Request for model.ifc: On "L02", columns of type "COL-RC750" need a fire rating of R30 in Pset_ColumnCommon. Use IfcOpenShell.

First a look at what the model holds.

```python
import ifcopenshell
import ifcopenshell.util.element

model = ifcopenshell.open("model.ifc")
print(model.schema)
storey = next(s for s in model.by_type("IfcBuildingStorey") if s.Name == "L02")
columns = [e for e in ifcopenshell.util.element.get_decomposition(storey) if e.is_a("IfcColumn")]
seen = {}
for e in columns:
    element_type = ifcopenshell.util.element.get_type(e)
    key = (element_type.Name if element_type != e and element_type else None, ifcopenshell.util.element.get_pset(e, "Pset_ColumnCommon", "FireRating"))
    seen[key] = seen.get(key, 0) + 1
for (name, value), count in sorted(seen.items(), key=str):
    print(count, "x", name, "|", value)
```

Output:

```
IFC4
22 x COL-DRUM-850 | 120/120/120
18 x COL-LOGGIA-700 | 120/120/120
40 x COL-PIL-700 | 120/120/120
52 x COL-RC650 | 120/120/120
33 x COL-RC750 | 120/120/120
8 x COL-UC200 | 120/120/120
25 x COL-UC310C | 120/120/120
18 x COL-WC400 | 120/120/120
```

```python
import ifcopenshell
import ifcopenshell.api.pset
import ifcopenshell.util.element

model = ifcopenshell.open("model.ifc")

storey = next(s for s in model.by_type("IfcBuildingStorey") if s.Name == "L02")
columns = [e for e in ifcopenshell.util.element.get_decomposition(storey) if e.is_a("IfcColumn")]

count = 0
for e in columns:
    element_type = ifcopenshell.util.element.get_type(e)
    if element_type in (None, e) or element_type.Name != "COL-RC750":
        continue
    # add_pset returns the element's existing set when there is one.
    pset = ifcopenshell.api.pset.add_pset(model, product=e, name="Pset_ColumnCommon")
    ifcopenshell.api.pset.edit_pset(model, pset=pset, properties={"FireRating": "R30"})
    count += 1

print(count, "columns updated")

model.write("model_rev.ifc")
```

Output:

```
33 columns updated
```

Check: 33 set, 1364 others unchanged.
